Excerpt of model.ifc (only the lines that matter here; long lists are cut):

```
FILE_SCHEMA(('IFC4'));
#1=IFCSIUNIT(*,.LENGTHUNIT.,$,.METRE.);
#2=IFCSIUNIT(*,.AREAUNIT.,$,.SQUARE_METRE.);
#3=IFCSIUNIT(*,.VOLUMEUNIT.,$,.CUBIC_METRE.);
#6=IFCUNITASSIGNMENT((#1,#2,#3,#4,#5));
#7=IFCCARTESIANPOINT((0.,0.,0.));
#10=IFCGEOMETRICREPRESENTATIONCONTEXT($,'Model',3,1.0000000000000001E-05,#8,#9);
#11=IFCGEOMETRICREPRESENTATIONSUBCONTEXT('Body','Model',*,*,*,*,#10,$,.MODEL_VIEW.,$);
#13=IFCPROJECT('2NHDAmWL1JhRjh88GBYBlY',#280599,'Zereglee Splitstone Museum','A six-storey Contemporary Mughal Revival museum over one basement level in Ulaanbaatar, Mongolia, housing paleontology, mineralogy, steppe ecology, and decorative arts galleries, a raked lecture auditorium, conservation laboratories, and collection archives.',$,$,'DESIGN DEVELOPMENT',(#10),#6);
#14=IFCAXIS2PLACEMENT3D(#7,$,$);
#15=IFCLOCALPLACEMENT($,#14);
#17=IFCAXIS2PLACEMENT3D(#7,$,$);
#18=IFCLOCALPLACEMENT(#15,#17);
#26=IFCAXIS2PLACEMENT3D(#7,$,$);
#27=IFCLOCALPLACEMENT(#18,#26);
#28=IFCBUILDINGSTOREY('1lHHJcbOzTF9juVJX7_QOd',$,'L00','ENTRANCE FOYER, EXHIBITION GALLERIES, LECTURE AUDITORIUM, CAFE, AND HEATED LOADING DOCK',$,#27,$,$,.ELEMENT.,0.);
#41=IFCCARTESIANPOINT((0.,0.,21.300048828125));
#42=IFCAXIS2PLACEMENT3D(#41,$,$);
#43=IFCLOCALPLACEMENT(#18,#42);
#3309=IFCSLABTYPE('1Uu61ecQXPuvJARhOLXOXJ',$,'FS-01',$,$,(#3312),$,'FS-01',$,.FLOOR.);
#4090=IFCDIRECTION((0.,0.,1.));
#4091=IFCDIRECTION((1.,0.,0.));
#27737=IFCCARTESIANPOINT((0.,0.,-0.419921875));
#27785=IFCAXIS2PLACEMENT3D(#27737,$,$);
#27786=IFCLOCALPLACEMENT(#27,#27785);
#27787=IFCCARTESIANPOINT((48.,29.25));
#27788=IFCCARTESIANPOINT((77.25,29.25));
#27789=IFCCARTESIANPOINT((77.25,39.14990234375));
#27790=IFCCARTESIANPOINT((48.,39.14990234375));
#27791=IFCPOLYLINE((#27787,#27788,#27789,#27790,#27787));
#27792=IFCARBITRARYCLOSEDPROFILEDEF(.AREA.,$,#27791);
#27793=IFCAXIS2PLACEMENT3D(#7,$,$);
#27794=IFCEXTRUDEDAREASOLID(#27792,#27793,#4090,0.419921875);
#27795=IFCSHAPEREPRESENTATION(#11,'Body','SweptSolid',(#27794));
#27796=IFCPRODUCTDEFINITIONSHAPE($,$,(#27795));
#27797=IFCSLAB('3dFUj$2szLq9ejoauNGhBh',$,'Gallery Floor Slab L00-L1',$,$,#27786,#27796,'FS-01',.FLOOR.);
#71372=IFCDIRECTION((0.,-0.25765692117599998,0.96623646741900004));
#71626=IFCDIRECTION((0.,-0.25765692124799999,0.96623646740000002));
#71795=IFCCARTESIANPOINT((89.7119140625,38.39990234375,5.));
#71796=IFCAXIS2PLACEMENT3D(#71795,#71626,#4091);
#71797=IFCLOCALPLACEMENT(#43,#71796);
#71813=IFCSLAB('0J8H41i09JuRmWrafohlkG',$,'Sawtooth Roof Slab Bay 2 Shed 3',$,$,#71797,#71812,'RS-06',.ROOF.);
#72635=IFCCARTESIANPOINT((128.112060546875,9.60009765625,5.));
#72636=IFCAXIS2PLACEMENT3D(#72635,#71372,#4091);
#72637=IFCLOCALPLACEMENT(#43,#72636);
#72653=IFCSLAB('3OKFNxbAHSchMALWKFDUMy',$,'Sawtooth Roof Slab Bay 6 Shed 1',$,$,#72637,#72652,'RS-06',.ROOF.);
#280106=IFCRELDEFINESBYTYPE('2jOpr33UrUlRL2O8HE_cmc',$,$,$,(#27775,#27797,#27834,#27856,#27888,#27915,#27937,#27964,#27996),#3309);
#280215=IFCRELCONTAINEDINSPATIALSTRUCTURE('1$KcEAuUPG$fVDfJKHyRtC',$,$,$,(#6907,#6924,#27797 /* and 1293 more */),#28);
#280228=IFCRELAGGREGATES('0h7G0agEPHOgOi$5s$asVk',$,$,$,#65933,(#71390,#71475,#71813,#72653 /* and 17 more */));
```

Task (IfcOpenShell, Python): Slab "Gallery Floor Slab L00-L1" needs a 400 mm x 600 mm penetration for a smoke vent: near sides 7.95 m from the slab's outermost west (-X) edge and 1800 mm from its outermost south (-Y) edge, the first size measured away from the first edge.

```python
import numpy as np
import ifcopenshell
import ifcopenshell.api.feature
import ifcopenshell.api.geometry
import ifcopenshell.api.root
import ifcopenshell.geom
import ifcopenshell.util.placement
import ifcopenshell.util.representation
import ifcopenshell.util.shape
import ifcopenshell.util.unit

model = ifcopenshell.open("model.ifc")
unit_scale = ifcopenshell.util.unit.calculate_unit_scale(model)
settings = ifcopenshell.geom.settings()


def volume(element):
    """Net volume in cubic metres, openings subtracted."""
    shape = ifcopenshell.geom.create_shape(settings, element)
    return ifcopenshell.util.shape.get_volume(shape.geometry)


slab = model.by_guid("3dFUj$2szLq9ejoauNGhBh")
before = volume(slab)

# Extent in the slab's own axes, in metres. The edges named are its -X and -Y sides.
slab_shape = ifcopenshell.geom.create_shape(settings, slab)
vertices = ifcopenshell.util.shape.get_vertices(slab_shape.geometry)
x_min, y_min, bottom = vertices.min(axis=0)
top = vertices[:, 2].max()

opening = ifcopenshell.api.root.create_entity(model, ifc_class="IfcOpeningElement", name="Smoke vent opening", predefined_type="OPENING")
context = ifcopenshell.util.representation.get_context(model, "Model", "Body", "MODEL_VIEW")
width, depth = 0.4, 0.6
outline = [(0.0, 0.0), (width, 0.0), (width, depth), (0.0, depth), (0.0, 0.0)]
# Overshoot both faces by 50 mm so the cut is clean.
shape = ifcopenshell.api.geometry.add_slab_representation(
    model, context=context, depth=top - bottom + 0.1, polyline=outline
)
ifcopenshell.api.geometry.assign_representation(model, product=opening, representation=shape)

matrix = ifcopenshell.util.placement.get_local_placement(slab.ObjectPlacement)
matrix[:, 3] = matrix @ np.append(np.array([x_min + 7.95, y_min + 1.8, bottom - 0.05]) / unit_scale, 1.0)
ifcopenshell.api.geometry.edit_object_placement(model, product=opening, matrix=matrix, is_si=False)
ifcopenshell.api.feature.add_feature(model, feature=opening, element=slab)

after = volume(slab)

print(f"slab volume {before:.3f} -> {after:.3f} m3")

model.write("model_edited.ifc")
```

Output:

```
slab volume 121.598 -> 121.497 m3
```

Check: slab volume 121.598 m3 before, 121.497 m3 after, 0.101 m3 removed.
